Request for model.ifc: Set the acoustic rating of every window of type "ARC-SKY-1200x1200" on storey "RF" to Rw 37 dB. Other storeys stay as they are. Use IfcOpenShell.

First a look at what the model holds.

```python
import ifcopenshell
import ifcopenshell.util.element

model = ifcopenshell.open("model.ifc")
print(model.schema)
storey = next(s for s in model.by_type("IfcBuildingStorey") if s.Name == "RF")
windows = [e for e in ifcopenshell.util.element.get_decomposition(storey) if e.is_a("IfcWindow")]
seen = {}
for e in windows:
    element_type = ifcopenshell.util.element.get_type(e)
    key = (element_type.Name if element_type != e and element_type else None, ifcopenshell.util.element.get_pset(e, "Pset_WindowCommon", "AcousticRating"))
    seen[key] = seen.get(key, 0) + 1
for (name, value), count in sorted(seen.items(), key=str):
    print(count, "x", name, "|", value)
```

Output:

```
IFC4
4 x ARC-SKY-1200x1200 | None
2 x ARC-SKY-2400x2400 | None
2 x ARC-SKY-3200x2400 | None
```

```python
import ifcopenshell
import ifcopenshell.api.pset
import ifcopenshell.util.element

model = ifcopenshell.open("model.ifc")

storey = next(s for s in model.by_type("IfcBuildingStorey") if s.Name == "RF")
windows = [e for e in ifcopenshell.util.element.get_decomposition(storey) if e.is_a("IfcWindow")]

count = 0
for e in windows:
    element_type = ifcopenshell.util.element.get_type(e)
    if element_type in (None, e) or element_type.Name != "ARC-SKY-1200x1200":
        continue
    found = ifcopenshell.util.element.get_pset(e, "Pset_WindowCommon", should_inherit=False)
    if found:
        pset = model.by_id(found["id"])
        if len(ifcopenshell.util.element.get_elements_by_pset(pset)) > 1:
            pset = ifcopenshell.api.pset.unshare_pset(model, products=[e], pset=pset)[0]
    else:
        pset = ifcopenshell.api.pset.add_pset(model, product=e, name="Pset_WindowCommon")
    ifcopenshell.api.pset.edit_pset(model, pset=pset, properties={"AcousticRating": "Rw 37 dB"})
    count += 1

print(count, "windows updated")

model.write("model_updated.ifc")
```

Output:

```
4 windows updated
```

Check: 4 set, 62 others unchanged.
